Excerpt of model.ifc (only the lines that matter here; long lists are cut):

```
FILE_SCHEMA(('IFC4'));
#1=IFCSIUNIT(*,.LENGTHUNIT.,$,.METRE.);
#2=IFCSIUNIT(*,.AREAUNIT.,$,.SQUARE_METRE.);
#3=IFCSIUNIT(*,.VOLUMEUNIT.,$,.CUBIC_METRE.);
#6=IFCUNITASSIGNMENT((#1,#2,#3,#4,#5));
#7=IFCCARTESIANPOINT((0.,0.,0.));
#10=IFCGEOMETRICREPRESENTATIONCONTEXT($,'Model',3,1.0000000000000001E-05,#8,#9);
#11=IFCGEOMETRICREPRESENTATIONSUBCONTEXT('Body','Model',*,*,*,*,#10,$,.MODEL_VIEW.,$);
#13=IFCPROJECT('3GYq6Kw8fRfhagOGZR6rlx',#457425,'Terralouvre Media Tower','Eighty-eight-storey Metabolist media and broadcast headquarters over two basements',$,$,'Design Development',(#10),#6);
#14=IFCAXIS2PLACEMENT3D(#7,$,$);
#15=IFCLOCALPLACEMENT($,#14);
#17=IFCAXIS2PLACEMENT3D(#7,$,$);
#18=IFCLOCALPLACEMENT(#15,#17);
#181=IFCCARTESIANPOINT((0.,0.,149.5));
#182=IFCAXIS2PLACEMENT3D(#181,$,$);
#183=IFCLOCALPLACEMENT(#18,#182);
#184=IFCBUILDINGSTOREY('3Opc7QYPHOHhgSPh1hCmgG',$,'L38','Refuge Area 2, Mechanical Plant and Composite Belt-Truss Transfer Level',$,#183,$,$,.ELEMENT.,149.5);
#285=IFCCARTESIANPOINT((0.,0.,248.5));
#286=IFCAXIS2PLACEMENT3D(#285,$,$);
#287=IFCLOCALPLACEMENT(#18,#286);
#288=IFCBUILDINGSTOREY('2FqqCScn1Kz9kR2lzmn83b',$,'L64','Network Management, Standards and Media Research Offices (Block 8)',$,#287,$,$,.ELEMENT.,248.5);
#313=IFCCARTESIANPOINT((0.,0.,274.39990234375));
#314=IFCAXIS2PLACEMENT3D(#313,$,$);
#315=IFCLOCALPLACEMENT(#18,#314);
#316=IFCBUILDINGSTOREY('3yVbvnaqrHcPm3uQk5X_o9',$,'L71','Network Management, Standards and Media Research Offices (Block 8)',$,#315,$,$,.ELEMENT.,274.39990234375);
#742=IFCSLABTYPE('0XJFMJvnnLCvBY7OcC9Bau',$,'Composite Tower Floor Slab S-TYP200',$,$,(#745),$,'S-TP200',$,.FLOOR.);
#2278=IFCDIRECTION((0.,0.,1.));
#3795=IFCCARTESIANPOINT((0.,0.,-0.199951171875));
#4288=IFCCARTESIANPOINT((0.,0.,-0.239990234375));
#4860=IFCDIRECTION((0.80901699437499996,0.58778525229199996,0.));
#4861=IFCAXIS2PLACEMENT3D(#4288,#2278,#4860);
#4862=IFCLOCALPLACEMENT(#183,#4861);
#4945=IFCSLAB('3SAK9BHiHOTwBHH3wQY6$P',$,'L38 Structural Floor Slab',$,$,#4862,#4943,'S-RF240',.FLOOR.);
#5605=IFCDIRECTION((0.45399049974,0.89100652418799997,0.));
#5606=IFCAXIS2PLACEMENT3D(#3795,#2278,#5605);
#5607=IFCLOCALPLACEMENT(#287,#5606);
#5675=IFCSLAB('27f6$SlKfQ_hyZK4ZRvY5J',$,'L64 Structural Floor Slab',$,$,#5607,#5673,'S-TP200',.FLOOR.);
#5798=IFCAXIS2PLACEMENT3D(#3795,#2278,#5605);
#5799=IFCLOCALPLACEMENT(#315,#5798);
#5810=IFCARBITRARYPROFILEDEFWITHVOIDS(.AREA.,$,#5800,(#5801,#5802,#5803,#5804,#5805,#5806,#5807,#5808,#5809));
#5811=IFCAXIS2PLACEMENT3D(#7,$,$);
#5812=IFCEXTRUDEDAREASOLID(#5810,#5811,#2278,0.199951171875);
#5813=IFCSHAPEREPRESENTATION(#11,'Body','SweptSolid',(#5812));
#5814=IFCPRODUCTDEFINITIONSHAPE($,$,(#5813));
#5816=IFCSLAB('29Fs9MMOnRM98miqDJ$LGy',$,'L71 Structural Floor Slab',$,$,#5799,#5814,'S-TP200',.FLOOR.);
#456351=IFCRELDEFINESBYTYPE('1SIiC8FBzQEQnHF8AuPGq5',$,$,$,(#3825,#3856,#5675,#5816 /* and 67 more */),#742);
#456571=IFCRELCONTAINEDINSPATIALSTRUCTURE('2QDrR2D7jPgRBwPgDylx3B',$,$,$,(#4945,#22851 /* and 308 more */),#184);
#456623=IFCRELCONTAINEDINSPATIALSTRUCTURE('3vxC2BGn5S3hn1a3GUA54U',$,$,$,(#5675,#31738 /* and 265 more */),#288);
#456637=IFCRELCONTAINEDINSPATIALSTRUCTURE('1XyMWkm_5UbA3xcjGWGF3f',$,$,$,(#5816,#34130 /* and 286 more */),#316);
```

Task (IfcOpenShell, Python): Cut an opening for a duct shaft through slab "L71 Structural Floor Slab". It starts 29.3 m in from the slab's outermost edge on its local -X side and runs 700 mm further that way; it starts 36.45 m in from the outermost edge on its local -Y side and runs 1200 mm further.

```python
import numpy as np
import ifcopenshell
import ifcopenshell.api.feature
import ifcopenshell.api.geometry
import ifcopenshell.api.root
import ifcopenshell.geom
import ifcopenshell.util.placement
import ifcopenshell.util.representation
import ifcopenshell.util.shape
import ifcopenshell.util.unit

model = ifcopenshell.open("model.ifc")
unit_scale = ifcopenshell.util.unit.calculate_unit_scale(model)
settings = ifcopenshell.geom.settings()


def volume(element):
    """Net volume in cubic metres, openings subtracted."""
    shape = ifcopenshell.geom.create_shape(settings, element)
    return ifcopenshell.util.shape.get_volume(shape.geometry)


slab = model.by_guid("29Fs9MMOnRM98miqDJ$LGy")
before = volume(slab)

# Extent in the slab's own axes, in metres. The edges named are its -X and -Y sides.
slab_shape = ifcopenshell.geom.create_shape(settings, slab)
vertices = ifcopenshell.util.shape.get_vertices(slab_shape.geometry)
x_min, y_min, bottom = vertices.min(axis=0)
top = vertices[:, 2].max()

opening = ifcopenshell.api.root.create_entity(model, ifc_class="IfcOpeningElement", name="Duct shaft opening", predefined_type="OPENING")
context = ifcopenshell.util.representation.get_context(model, "Model", "Body", "MODEL_VIEW")
width, depth = 0.7, 1.2
outline = [(0.0, 0.0), (width, 0.0), (width, depth), (0.0, depth), (0.0, 0.0)]
# Overshoot both faces by 50 mm so the cut is clean.
shape = ifcopenshell.api.geometry.add_slab_representation(
    model, context=context, depth=top - bottom + 0.1, polyline=outline
)
ifcopenshell.api.geometry.assign_representation(model, product=opening, representation=shape)

matrix = ifcopenshell.util.placement.get_local_placement(slab.ObjectPlacement)
matrix[:, 3] = matrix @ np.append(np.array([x_min + 29.3, y_min + 36.45, bottom - 0.05]) / unit_scale, 1.0)
ifcopenshell.api.geometry.edit_object_placement(model, product=opening, matrix=matrix, is_si=False)
ifcopenshell.api.feature.add_feature(model, feature=opening, element=slab)

after = volume(slab)

print(f"slab volume {before:.3f} -> {after:.3f} m3")

model.write("model_updated.ifc")
```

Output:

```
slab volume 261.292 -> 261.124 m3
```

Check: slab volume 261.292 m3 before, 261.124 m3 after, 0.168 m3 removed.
